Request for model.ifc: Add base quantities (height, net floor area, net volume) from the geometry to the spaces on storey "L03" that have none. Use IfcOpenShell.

First a look at what the model holds.

```python
import ifcopenshell
import ifcopenshell.util.element
import ifcopenshell.util.unit

model = ifcopenshell.open("model.ifc")
print(model.schema)
for unit_type in ("LENGTHUNIT", "AREAUNIT", "VOLUMEUNIT"):
    print(unit_type, ifcopenshell.util.unit.calculate_unit_scale(model, unit_type))
storey = next(s for s in model.by_type("IfcBuildingStorey") if s.Name == "L03")
spaces = [e for e in ifcopenshell.util.element.get_decomposition(storey) if e.is_a("IfcSpace")]
for e in sorted(spaces, key=lambda e: e.id()):
    print(e.id(), e.is_a(), e.Name, list(ifcopenshell.util.element.get_psets(e, qtos_only=True)), sep=" | ")
```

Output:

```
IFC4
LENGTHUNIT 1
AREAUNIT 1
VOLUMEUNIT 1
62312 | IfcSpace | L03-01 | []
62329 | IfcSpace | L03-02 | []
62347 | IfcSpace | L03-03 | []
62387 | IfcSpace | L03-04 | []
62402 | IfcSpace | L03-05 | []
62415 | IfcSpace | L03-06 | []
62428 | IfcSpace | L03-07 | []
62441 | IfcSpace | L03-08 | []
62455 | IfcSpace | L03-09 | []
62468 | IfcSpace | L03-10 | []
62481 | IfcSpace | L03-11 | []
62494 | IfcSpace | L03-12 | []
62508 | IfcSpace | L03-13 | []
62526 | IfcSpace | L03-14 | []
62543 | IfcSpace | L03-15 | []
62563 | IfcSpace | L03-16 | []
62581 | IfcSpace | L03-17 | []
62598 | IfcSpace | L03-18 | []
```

```python
import ifcopenshell
import ifcopenshell.api.pset
import ifcopenshell.geom
import ifcopenshell.util.element
import ifcopenshell.util.shape
import ifcopenshell.util.unit

model = ifcopenshell.open("model.ifc")
unit_scale = ifcopenshell.util.unit.calculate_unit_scale(model)
area_scale = ifcopenshell.util.unit.calculate_unit_scale(model, "AREAUNIT")
volume_scale = ifcopenshell.util.unit.calculate_unit_scale(model, "VOLUMEUNIT")
settings = ifcopenshell.geom.settings()

storey = next(s for s in model.by_type("IfcBuildingStorey") if s.Name == "L03")
spaces = [e for e in ifcopenshell.util.element.get_decomposition(storey) if e.is_a("IfcSpace")]

for e in sorted(spaces, key=lambda e: e.id()):
    if ifcopenshell.util.element.get_psets(e, qtos_only=True, should_inherit=False):
        continue
    # Geometry comes back in metres, in the element's own axes.
    shape = ifcopenshell.geom.create_shape(settings, e)
    values = {
        "Height": ifcopenshell.util.shape.get_z(shape.geometry) / unit_scale,
        "NetFloorArea": ifcopenshell.util.shape.get_footprint_area(shape.geometry) / area_scale,
        "NetVolume": ifcopenshell.util.shape.get_volume(shape.geometry) / volume_scale,
    }
    qto = ifcopenshell.api.pset.add_qto(model, product=e, name="Qto_SpaceBaseQuantities")
    ifcopenshell.api.pset.edit_qto(model, qto=qto, properties=values)
    print(e.id(), {k: round(v, 3) for k, v in values.items()})

model.write("model_edited.ifc")
```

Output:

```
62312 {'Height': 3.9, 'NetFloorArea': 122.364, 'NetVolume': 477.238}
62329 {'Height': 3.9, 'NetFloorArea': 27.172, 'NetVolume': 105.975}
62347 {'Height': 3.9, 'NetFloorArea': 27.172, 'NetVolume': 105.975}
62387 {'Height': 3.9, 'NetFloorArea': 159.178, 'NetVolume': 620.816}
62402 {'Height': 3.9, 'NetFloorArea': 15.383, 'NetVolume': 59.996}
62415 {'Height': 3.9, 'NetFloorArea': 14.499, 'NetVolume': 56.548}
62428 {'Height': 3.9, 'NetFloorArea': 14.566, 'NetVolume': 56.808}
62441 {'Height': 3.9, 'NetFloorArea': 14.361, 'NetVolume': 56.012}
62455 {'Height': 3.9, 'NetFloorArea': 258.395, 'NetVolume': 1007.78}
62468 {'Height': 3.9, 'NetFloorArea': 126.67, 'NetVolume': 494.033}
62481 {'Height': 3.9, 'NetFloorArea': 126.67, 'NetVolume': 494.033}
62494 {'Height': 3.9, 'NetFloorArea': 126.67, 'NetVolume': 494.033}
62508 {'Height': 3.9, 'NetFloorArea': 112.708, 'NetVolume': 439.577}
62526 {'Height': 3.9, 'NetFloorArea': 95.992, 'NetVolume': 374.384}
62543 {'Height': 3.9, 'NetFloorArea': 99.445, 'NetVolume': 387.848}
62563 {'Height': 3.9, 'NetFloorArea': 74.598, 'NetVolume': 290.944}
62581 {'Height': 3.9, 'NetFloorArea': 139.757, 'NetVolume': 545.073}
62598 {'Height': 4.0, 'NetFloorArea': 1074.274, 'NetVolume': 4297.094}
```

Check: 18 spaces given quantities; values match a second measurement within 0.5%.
